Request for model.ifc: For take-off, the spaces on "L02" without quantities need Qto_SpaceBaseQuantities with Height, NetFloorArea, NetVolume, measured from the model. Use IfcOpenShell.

First a look at what the model holds.

```python
import ifcopenshell
import ifcopenshell.util.element
import ifcopenshell.util.unit

model = ifcopenshell.open("model.ifc")
print(model.schema)
for unit_type in ("LENGTHUNIT", "AREAUNIT", "VOLUMEUNIT"):
    print(unit_type, ifcopenshell.util.unit.calculate_unit_scale(model, unit_type))
storey = next(s for s in model.by_type("IfcBuildingStorey") if s.Name == "L02")
spaces = [e for e in ifcopenshell.util.element.get_decomposition(storey) if e.is_a("IfcSpace")]
for e in sorted(spaces, key=lambda e: e.id()):
    print(e.id(), e.is_a(), e.Name, list(ifcopenshell.util.element.get_psets(e, qtos_only=True)), sep=" | ")
```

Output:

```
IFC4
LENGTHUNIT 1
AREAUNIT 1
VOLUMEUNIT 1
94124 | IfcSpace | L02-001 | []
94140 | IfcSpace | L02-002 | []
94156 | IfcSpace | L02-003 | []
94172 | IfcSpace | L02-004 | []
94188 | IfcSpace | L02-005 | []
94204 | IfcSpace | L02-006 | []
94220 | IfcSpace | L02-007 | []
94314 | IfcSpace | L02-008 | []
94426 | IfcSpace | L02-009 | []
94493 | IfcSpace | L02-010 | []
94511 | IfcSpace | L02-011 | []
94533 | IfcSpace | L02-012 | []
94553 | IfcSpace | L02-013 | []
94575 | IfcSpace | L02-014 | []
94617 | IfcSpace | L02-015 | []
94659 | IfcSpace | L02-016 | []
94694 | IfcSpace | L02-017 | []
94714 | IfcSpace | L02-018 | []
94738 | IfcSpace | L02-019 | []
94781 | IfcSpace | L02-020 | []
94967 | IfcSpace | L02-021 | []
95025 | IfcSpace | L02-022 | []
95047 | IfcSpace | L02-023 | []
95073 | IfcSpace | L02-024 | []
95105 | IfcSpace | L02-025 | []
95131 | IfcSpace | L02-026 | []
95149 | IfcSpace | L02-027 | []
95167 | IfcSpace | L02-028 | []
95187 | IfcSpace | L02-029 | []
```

```python
import ifcopenshell
import ifcopenshell.api.pset
import ifcopenshell.geom
import ifcopenshell.util.element
import ifcopenshell.util.shape
import ifcopenshell.util.unit

model = ifcopenshell.open("model.ifc")
unit_scale = ifcopenshell.util.unit.calculate_unit_scale(model)
area_scale = ifcopenshell.util.unit.calculate_unit_scale(model, "AREAUNIT")
volume_scale = ifcopenshell.util.unit.calculate_unit_scale(model, "VOLUMEUNIT")
settings = ifcopenshell.geom.settings()

storey = next(s for s in model.by_type("IfcBuildingStorey") if s.Name == "L02")
spaces = [e for e in ifcopenshell.util.element.get_decomposition(storey) if e.is_a("IfcSpace")]

for e in sorted(spaces, key=lambda e: e.id()):
    if ifcopenshell.util.element.get_psets(e, qtos_only=True, should_inherit=False):
        continue
    # Geometry comes back in metres, in the element's own axes.
    shape = ifcopenshell.geom.create_shape(settings, e)
    values = {
        "Height": ifcopenshell.util.shape.get_z(shape.geometry) / unit_scale,
        "NetFloorArea": ifcopenshell.util.shape.get_footprint_area(shape.geometry) / area_scale,
        "NetVolume": ifcopenshell.util.shape.get_volume(shape.geometry) / volume_scale,
    }
    qto = ifcopenshell.api.pset.add_qto(model, product=e, name="Qto_SpaceBaseQuantities")
    ifcopenshell.api.pset.edit_qto(model, qto=qto, properties=values)
    print(e.id(), {k: round(v, 3) for k, v in values.items()})

model.write("model_v2.ifc")
```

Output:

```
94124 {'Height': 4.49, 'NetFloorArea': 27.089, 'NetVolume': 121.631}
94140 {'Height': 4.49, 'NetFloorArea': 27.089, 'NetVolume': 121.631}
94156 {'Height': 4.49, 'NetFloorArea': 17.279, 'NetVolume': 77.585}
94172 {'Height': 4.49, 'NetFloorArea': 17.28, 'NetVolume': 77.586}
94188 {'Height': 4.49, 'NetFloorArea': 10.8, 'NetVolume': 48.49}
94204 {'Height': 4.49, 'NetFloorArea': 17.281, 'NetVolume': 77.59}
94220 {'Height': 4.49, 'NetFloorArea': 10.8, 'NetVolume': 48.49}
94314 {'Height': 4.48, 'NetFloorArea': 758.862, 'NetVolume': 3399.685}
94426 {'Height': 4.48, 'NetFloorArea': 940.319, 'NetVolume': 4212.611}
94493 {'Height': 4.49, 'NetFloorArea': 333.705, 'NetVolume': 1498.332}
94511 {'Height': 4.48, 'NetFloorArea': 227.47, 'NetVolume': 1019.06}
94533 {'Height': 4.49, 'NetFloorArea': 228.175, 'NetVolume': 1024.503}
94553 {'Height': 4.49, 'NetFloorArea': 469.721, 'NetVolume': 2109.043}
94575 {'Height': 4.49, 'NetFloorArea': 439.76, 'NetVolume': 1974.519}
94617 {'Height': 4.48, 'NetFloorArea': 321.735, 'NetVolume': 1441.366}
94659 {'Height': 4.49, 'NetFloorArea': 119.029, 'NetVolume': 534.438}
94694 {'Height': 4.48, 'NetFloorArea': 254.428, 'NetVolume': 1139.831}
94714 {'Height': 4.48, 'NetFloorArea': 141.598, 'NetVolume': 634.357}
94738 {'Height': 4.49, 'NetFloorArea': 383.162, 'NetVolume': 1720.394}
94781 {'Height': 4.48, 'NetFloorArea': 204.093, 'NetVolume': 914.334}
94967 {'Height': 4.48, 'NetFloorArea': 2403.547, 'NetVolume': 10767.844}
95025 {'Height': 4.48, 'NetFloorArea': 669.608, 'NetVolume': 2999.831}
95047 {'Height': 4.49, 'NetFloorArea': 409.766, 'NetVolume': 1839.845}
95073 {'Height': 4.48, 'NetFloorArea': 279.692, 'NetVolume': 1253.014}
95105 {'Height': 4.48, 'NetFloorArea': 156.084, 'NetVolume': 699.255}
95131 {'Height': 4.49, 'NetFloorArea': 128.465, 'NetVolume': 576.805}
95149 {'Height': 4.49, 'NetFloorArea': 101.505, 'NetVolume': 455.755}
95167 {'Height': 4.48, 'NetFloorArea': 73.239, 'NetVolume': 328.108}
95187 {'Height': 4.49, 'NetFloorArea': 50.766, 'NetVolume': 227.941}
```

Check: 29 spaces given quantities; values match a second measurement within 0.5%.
